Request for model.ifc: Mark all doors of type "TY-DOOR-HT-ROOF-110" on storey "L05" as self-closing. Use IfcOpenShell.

First a look at what the model holds.

```python
import ifcopenshell
import ifcopenshell.util.element

model = ifcopenshell.open("model.ifc")
print(model.schema)
storey = next(s for s in model.by_type("IfcBuildingStorey") if s.Name == "L05")
doors = [e for e in ifcopenshell.util.element.get_decomposition(storey) if e.is_a("IfcDoor")]
seen = {}
for e in doors:
    element_type = ifcopenshell.util.element.get_type(e)
    key = (element_type.Name if element_type != e and element_type else None, ifcopenshell.util.element.get_pset(e, "Pset_DoorCommon", "SelfClosing"))
    seen[key] = seen.get(key, 0) + 1
for (name, value), count in sorted(seen.items(), key=str):
    print(count, "x", name, "|", value)
```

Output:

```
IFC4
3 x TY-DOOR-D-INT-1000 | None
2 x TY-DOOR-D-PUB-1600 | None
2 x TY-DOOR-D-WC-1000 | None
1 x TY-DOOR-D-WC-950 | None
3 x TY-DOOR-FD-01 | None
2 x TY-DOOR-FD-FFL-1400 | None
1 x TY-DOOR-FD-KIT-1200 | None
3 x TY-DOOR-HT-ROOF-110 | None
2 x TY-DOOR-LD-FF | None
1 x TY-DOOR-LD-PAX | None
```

```python
import ifcopenshell
import ifcopenshell.api.pset
import ifcopenshell.util.element

model = ifcopenshell.open("model.ifc")

storey = next(s for s in model.by_type("IfcBuildingStorey") if s.Name == "L05")
doors = [e for e in ifcopenshell.util.element.get_decomposition(storey) if e.is_a("IfcDoor")]

count = 0
for e in doors:
    element_type = ifcopenshell.util.element.get_type(e)
    if element_type in (None, e) or element_type.Name != "TY-DOOR-HT-ROOF-110":
        continue
    # add_pset returns the element's existing set when there is one.
    pset = ifcopenshell.api.pset.add_pset(model, product=e, name="Pset_DoorCommon")
    ifcopenshell.api.pset.edit_pset(model, pset=pset, properties={"SelfClosing": True})
    count += 1

print(count, "doors updated")

model.write("model-out.ifc")
```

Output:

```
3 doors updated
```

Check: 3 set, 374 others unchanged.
